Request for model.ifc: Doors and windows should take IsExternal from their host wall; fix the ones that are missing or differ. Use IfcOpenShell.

First a look at what the model holds.

```python
import ifcopenshell
import ifcopenshell.util.element

model = ifcopenshell.open("model.ifc")
print(model.schema)
seen = {}
for e in model.by_type("IfcDoor") + model.by_type("IfcWindow"):
    if not e.FillsVoids:
        continue
    host = e.FillsVoids[0].RelatingOpeningElement.VoidsElements[0].RelatingBuildingElement
    own = ifcopenshell.util.element.get_pset(e, f"Pset_{e.is_a()[3:].removesuffix('StandardCase')}Common", "IsExternal")
    wall = ifcopenshell.util.element.get_pset(host, "Pset_WallCommon", "IsExternal")
    seen[e.is_a(), own, wall] = seen.get((e.is_a(), own, wall), 0) + 1
for (cls, own, wall), count in sorted(seen.items(), key=str):
    print(count, cls, "IsExternal:", own, "| host wall:", wall)
```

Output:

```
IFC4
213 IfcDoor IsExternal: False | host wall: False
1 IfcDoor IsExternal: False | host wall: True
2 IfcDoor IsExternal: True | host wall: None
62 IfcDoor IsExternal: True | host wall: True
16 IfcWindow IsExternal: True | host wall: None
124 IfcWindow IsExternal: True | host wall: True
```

```python
import ifcopenshell
import ifcopenshell.api.pset
import ifcopenshell.util.element

model = ifcopenshell.open("model.ifc")

count = 0
for ifc_class, pset_name in (("IfcDoor", "Pset_DoorCommon"), ("IfcWindow", "Pset_WindowCommon")):
    for e in model.by_type(ifc_class):
        if not e.FillsVoids:
            continue
        host = e.FillsVoids[0].RelatingOpeningElement.VoidsElements[0].RelatingBuildingElement
        external = ifcopenshell.util.element.get_pset(host, "Pset_WallCommon", "IsExternal")
        if external is None or ifcopenshell.util.element.get_pset(e, pset_name, "IsExternal") == external:
            continue
        pset = ifcopenshell.api.pset.add_pset(model, product=e, name=pset_name)
        ifcopenshell.api.pset.edit_pset(model, pset=pset, properties={"IsExternal": external})
        count += 1

print(count, "updated")

model.write("model_edited.ifc")
```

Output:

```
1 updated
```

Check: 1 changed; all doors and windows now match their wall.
